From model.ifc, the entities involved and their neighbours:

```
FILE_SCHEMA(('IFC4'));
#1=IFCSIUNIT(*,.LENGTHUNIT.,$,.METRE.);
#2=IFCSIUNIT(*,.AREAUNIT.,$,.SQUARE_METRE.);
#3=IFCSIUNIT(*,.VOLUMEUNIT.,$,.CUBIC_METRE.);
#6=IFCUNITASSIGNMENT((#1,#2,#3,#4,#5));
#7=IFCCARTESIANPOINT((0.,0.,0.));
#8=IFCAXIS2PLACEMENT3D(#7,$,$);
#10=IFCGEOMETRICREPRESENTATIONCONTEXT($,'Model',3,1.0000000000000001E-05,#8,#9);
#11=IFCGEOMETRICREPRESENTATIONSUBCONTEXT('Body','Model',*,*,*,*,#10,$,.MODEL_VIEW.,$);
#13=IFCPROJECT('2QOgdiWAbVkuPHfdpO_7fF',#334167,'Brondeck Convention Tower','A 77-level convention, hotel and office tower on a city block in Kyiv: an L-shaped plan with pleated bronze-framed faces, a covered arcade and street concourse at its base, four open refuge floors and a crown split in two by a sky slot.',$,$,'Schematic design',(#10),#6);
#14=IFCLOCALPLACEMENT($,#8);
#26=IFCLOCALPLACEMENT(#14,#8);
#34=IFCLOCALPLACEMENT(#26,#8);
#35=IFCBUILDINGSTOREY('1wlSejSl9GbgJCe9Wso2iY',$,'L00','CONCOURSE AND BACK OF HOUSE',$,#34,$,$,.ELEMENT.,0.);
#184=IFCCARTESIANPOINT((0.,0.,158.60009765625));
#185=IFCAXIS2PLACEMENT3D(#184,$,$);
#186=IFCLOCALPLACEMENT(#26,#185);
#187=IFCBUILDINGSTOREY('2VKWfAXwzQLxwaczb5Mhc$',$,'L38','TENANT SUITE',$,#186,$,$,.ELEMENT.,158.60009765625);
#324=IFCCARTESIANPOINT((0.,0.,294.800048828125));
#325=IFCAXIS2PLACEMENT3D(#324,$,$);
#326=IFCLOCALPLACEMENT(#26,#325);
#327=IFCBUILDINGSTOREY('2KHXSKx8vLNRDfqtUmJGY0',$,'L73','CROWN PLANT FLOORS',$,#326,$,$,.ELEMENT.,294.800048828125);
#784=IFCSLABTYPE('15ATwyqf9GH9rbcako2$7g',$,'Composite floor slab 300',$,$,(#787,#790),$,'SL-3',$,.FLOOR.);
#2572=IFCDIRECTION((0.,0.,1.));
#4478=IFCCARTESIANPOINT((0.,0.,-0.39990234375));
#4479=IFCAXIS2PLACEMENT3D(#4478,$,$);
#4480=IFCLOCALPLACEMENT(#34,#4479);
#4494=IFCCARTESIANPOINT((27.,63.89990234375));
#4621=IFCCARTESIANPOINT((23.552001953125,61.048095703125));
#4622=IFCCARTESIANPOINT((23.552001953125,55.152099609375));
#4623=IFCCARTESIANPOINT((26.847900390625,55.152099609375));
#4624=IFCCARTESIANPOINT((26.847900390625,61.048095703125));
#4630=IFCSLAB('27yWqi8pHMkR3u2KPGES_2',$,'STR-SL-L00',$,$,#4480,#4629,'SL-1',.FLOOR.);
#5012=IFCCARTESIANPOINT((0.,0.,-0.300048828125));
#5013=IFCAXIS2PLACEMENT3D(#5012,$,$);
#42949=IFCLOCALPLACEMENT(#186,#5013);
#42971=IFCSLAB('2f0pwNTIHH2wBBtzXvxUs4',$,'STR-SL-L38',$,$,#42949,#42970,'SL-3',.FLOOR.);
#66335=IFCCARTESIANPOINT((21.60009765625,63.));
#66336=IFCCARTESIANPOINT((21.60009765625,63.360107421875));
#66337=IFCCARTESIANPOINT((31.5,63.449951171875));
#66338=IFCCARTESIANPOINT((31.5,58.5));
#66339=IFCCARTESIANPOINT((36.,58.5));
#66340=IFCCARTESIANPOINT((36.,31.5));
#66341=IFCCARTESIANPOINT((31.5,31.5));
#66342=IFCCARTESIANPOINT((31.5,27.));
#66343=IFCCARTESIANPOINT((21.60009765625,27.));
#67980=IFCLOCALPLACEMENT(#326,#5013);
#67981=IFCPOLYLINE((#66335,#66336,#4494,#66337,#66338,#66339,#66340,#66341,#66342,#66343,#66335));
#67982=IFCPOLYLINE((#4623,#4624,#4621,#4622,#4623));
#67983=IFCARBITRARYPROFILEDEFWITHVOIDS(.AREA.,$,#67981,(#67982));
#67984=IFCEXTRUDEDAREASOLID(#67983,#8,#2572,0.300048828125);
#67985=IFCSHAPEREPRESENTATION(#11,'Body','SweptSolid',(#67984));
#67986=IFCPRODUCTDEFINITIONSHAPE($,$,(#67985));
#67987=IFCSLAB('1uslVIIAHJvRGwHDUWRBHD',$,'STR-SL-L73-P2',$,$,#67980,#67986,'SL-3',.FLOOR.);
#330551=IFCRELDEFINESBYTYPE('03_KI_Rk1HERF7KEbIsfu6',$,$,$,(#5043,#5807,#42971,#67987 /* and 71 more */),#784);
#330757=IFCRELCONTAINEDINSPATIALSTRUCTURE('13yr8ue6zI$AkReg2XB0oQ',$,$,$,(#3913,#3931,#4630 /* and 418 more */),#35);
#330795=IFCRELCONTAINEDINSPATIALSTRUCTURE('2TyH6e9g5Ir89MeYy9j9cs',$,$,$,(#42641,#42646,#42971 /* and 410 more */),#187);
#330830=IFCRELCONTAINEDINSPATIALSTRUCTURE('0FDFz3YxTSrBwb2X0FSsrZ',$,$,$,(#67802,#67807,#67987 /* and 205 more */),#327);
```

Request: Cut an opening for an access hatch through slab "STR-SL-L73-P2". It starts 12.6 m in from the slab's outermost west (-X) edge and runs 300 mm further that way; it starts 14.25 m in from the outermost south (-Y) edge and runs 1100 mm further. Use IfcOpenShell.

```python
import numpy as np
import ifcopenshell
import ifcopenshell.api.feature
import ifcopenshell.api.geometry
import ifcopenshell.api.root
import ifcopenshell.geom
import ifcopenshell.util.placement
import ifcopenshell.util.representation
import ifcopenshell.util.shape
import ifcopenshell.util.unit

model = ifcopenshell.open("model.ifc")
unit_scale = ifcopenshell.util.unit.calculate_unit_scale(model)
settings = ifcopenshell.geom.settings()


def volume(element):
    """Net volume in cubic metres, openings subtracted."""
    shape = ifcopenshell.geom.create_shape(settings, element)
    return ifcopenshell.util.shape.get_volume(shape.geometry)


slab = model.by_guid("1uslVIIAHJvRGwHDUWRBHD")
before = volume(slab)

# Extent in the slab's own axes, in metres. The edges named are its -X and -Y sides.
slab_shape = ifcopenshell.geom.create_shape(settings, slab)
vertices = ifcopenshell.util.shape.get_vertices(slab_shape.geometry)
x_min, y_min, bottom = vertices.min(axis=0)
top = vertices[:, 2].max()

opening = ifcopenshell.api.root.create_entity(model, ifc_class="IfcOpeningElement", name="Access hatch opening", predefined_type="OPENING")
context = ifcopenshell.util.representation.get_context(model, "Model", "Body", "MODEL_VIEW")
width, depth = 0.3, 1.1
outline = [(0.0, 0.0), (width, 0.0), (width, depth), (0.0, depth), (0.0, 0.0)]
# Overshoot both faces by 50 mm so the cut is clean.
shape = ifcopenshell.api.geometry.add_slab_representation(
    model, context=context, depth=top - bottom + 0.1, polyline=outline
)
ifcopenshell.api.geometry.assign_representation(model, product=opening, representation=shape)

matrix = ifcopenshell.util.placement.get_local_placement(slab.ObjectPlacement)
matrix[:, 3] = matrix @ np.append(np.array([x_min + 12.6, y_min + 14.25, bottom - 0.05]) / unit_scale, 1.0)
ifcopenshell.api.geometry.edit_object_placement(model, product=opening, matrix=matrix, is_si=False)
ifcopenshell.api.feature.add_feature(model, feature=opening, element=slab)

after = volume(slab)

print(f"slab volume {before:.3f} -> {after:.3f} m3")

model.write("model-out.ifc")
```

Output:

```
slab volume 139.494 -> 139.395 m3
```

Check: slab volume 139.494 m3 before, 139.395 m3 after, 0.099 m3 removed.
